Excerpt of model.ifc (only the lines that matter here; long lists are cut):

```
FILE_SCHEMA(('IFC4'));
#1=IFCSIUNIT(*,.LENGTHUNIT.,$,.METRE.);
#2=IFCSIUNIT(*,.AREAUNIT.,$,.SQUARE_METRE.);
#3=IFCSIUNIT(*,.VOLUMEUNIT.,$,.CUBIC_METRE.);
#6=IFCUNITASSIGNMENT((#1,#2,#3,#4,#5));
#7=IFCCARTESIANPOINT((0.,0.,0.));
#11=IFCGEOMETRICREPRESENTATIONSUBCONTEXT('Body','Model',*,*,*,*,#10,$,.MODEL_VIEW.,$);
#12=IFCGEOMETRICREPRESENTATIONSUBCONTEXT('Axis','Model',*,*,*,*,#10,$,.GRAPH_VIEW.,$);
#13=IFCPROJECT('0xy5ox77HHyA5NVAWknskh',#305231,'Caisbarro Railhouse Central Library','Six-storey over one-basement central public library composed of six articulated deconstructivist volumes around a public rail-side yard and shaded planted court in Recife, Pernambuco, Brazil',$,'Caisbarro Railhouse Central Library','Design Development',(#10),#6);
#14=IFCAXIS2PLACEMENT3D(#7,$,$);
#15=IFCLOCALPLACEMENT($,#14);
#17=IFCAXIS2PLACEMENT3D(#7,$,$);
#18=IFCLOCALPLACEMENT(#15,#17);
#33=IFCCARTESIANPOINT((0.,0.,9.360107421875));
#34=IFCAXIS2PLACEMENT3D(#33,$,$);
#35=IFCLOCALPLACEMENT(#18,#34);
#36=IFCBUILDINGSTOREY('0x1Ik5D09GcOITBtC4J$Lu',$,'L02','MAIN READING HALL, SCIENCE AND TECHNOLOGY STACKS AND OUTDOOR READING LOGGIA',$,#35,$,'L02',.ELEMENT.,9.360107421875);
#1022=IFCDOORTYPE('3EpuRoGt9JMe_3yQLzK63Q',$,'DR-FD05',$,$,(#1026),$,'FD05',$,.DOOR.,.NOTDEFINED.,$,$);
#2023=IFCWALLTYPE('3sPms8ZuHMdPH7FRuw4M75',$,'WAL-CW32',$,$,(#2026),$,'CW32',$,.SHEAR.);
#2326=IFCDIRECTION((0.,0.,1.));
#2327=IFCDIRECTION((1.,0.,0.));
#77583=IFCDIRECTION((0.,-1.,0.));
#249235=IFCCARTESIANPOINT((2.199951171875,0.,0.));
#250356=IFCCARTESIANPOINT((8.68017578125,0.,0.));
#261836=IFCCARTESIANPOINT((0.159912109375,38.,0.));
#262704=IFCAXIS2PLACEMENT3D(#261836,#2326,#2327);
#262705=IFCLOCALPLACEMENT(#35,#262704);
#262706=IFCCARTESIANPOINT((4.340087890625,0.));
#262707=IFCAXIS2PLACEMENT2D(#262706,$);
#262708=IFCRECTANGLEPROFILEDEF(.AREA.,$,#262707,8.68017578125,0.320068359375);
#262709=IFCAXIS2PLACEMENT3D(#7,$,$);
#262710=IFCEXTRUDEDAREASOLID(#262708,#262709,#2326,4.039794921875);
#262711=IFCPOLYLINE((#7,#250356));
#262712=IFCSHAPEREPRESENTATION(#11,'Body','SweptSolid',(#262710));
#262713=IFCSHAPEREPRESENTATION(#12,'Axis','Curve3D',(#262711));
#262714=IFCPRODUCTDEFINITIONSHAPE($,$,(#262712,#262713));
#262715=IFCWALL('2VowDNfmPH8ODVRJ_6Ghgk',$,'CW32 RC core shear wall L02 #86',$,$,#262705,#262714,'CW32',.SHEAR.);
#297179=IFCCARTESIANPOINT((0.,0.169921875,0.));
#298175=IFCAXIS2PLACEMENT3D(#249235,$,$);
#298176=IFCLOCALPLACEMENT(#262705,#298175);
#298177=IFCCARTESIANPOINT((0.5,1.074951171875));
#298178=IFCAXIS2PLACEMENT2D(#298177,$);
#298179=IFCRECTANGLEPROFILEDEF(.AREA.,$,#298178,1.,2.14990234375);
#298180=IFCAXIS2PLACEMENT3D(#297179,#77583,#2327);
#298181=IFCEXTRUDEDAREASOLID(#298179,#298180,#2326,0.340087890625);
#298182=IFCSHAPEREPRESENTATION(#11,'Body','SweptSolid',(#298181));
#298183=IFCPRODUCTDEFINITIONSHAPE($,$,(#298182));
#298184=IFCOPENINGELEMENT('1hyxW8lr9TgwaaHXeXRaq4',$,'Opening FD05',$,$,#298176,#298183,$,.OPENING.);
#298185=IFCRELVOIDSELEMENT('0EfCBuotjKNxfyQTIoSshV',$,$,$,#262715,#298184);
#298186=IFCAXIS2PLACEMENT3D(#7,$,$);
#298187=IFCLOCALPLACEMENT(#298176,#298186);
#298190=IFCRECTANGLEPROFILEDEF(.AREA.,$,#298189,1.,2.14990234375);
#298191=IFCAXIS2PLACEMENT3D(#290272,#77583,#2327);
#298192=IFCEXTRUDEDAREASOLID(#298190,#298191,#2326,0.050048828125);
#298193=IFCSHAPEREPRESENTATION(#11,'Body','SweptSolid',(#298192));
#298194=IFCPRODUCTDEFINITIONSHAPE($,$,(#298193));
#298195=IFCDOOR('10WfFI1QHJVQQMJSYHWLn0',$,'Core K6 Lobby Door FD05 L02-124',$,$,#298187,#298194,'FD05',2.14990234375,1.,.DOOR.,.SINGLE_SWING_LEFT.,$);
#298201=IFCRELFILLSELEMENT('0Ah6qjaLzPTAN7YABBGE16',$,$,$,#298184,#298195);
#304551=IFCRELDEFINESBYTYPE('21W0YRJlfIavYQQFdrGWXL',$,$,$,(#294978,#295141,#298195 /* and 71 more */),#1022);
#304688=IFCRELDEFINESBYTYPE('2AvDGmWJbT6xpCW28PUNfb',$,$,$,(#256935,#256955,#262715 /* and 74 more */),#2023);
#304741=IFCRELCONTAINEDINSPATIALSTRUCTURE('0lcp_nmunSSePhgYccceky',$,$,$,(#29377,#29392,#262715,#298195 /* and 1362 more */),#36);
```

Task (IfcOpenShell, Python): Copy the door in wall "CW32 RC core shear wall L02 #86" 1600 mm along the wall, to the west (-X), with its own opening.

```python
import ifcopenshell
import ifcopenshell.api.feature
import ifcopenshell.api.geometry
import ifcopenshell.api.root
import ifcopenshell.geom
import ifcopenshell.util.element
import ifcopenshell.util.placement
import ifcopenshell.util.shape
import ifcopenshell.util.unit

model = ifcopenshell.open("model.ifc")
unit_scale = ifcopenshell.util.unit.calculate_unit_scale(model)
settings = ifcopenshell.geom.settings()


def volume(element):
    """Net volume in cubic metres, openings subtracted."""
    shape = ifcopenshell.geom.create_shape(settings, element)
    return ifcopenshell.util.shape.get_volume(shape.geometry)


door = model.by_id(298195)
opening = door.FillsVoids[0].RelatingOpeningElement
wall = opening.VoidsElements[0].RelatingBuildingElement
before = volume(wall)
shift = ifcopenshell.util.placement.get_local_placement(wall.ObjectPlacement)[:3, 0] * -1.6 / unit_scale

# copy_class copies the void relationship, type, container and properties, but no geometry.
new_opening = ifcopenshell.api.root.copy_class(model, product=opening)
new_opening.Representation = ifcopenshell.util.element.copy_deep(
    model, opening.Representation, exclude=["IfcGeometricRepresentationContext", "IfcRepresentationMap"]
)
new_door = ifcopenshell.api.root.copy_class(model, product=door)
new_door.Representation = ifcopenshell.util.element.copy_deep(
    model, door.Representation, exclude=["IfcGeometricRepresentationContext", "IfcRepresentationMap"]
)
new_door.Tag = None
ifcopenshell.api.feature.add_filling(model, opening=new_opening, element=new_door)

for old, new in ((opening, new_opening), (door, new_door)):
    matrix = ifcopenshell.util.placement.get_local_placement(old.ObjectPlacement)
    matrix[:3, 3] += shift
    ifcopenshell.api.geometry.edit_object_placement(model, product=new, matrix=matrix, is_si=False)

after = volume(wall)

print(f"wall volume {before:.3f} -> {after:.3f} m3")

model.write("model_updated.ifc")
```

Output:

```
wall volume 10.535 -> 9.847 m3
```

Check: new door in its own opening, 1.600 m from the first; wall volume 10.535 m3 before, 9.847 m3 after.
